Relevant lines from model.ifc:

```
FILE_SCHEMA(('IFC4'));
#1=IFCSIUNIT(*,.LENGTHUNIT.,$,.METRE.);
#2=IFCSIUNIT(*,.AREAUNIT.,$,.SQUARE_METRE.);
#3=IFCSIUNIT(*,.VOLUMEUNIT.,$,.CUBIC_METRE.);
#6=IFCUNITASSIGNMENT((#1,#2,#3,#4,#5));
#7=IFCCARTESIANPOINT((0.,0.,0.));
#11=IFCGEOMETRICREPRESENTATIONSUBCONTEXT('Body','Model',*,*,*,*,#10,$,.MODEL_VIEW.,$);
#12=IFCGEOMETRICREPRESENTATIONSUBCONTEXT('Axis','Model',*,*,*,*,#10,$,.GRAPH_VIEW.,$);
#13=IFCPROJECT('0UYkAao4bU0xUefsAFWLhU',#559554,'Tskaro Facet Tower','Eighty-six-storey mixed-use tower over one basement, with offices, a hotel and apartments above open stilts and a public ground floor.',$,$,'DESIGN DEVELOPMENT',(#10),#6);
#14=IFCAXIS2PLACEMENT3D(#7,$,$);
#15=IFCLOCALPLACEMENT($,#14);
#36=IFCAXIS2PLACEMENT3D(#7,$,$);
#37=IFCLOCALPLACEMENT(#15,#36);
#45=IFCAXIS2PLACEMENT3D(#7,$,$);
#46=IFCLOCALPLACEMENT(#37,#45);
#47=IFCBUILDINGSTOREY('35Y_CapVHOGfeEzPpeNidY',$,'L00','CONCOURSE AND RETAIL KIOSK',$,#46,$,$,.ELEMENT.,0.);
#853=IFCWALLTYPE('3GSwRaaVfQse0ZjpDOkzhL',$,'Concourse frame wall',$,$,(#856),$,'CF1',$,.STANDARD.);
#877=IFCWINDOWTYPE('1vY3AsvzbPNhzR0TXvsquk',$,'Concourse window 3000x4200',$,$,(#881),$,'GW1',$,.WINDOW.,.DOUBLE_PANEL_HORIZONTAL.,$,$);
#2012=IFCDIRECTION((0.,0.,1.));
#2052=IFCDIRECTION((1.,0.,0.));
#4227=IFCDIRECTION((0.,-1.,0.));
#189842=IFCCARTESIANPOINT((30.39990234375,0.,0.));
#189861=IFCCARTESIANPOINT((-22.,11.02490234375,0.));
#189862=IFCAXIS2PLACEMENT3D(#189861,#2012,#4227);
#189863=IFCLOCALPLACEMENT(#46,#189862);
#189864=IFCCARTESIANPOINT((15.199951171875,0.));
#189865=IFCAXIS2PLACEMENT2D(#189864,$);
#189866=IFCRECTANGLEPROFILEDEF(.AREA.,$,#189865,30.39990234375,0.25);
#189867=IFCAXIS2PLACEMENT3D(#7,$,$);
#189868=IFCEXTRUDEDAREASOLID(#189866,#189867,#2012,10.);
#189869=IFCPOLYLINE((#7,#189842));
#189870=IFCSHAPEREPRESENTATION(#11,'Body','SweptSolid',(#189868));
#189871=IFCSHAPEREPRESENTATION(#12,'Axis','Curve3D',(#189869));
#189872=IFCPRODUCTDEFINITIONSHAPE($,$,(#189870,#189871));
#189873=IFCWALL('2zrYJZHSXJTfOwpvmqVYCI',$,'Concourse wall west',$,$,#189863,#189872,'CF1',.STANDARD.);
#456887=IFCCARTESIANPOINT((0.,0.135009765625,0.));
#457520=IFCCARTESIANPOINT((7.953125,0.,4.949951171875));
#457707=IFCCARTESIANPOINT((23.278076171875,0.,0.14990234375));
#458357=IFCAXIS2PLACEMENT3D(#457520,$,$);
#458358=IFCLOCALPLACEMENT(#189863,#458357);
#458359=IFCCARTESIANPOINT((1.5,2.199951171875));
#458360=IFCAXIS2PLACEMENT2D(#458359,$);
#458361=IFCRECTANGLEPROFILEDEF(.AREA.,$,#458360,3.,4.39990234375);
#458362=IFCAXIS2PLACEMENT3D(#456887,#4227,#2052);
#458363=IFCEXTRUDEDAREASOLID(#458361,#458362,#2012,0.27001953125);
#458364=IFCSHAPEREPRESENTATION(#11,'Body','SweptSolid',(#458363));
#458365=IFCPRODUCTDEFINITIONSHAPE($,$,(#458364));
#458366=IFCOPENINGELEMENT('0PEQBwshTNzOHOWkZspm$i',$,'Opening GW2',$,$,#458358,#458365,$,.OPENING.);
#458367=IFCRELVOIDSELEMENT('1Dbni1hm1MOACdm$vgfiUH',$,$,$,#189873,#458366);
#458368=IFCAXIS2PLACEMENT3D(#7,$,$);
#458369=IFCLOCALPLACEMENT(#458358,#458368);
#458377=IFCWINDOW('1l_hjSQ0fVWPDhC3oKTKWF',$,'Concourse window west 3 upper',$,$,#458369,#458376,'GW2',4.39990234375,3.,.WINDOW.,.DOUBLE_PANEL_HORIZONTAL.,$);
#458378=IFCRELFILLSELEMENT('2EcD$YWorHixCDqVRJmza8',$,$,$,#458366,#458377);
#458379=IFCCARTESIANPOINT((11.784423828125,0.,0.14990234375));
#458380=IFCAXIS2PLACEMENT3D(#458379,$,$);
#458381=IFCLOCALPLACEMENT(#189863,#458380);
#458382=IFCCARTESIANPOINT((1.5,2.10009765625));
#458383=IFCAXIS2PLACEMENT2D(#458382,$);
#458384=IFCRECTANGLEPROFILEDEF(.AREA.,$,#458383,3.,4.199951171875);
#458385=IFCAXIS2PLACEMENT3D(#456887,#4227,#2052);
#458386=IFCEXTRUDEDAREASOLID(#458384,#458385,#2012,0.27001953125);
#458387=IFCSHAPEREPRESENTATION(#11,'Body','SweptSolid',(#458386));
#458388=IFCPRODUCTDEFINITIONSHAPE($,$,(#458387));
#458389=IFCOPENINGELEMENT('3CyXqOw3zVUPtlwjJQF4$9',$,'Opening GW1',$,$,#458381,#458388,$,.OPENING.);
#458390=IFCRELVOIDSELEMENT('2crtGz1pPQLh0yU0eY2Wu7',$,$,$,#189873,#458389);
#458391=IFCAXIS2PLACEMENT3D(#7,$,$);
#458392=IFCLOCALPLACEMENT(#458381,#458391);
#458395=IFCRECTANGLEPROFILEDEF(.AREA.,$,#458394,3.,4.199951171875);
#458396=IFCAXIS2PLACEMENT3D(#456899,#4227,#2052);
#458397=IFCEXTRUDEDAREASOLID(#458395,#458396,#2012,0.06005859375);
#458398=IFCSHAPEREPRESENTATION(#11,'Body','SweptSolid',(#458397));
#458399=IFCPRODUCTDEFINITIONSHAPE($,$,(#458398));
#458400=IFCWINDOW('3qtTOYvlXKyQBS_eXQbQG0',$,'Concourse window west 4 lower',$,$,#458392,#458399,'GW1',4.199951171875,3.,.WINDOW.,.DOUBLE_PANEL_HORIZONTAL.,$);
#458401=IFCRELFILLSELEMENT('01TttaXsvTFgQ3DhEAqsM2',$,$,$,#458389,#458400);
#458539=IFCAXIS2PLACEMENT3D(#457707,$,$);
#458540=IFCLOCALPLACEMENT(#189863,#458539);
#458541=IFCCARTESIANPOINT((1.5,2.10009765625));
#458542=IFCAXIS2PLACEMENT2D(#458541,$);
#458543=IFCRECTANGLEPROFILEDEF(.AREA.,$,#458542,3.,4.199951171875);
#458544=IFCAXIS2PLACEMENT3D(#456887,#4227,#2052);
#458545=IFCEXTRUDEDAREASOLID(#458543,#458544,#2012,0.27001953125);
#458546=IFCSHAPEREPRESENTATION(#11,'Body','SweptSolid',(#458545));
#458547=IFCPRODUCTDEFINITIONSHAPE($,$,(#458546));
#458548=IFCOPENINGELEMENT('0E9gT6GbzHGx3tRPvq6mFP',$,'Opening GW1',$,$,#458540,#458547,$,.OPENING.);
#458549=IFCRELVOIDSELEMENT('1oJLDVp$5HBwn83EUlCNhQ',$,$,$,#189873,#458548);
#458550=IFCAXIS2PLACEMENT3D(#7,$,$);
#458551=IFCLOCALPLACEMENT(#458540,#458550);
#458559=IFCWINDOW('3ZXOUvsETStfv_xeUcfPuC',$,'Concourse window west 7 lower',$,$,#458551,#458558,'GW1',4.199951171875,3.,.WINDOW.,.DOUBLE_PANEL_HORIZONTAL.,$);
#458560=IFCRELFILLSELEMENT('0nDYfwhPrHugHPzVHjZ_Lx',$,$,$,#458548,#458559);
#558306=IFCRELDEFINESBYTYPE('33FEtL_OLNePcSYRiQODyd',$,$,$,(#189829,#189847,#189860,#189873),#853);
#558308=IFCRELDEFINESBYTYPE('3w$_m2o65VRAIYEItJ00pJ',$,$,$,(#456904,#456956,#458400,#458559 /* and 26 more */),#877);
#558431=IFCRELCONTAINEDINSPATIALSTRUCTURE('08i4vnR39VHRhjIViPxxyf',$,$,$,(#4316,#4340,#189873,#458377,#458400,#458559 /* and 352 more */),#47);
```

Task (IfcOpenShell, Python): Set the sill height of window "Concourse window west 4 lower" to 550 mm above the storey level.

```python
import numpy as np
import ifcopenshell
import ifcopenshell.api.geometry
import ifcopenshell.geom
import ifcopenshell.util.element
import ifcopenshell.util.placement
import ifcopenshell.util.shape
import ifcopenshell.util.unit

model = ifcopenshell.open("model.ifc")
unit_scale = ifcopenshell.util.unit.calculate_unit_scale(model)

window = model.by_guid("3qtTOYvlXKyQBS_eXQbQG0")
opening = window.FillsVoids[0].RelatingOpeningElement
storey = ifcopenshell.util.element.get_container(window, ifc_class="IfcBuildingStorey")
level = ifcopenshell.util.placement.get_local_placement(storey.ObjectPlacement)[2, 3]

# The opening's origin need not be at the sill, so measure its lowest point.
shape = ifcopenshell.geom.create_shape(ifcopenshell.geom.settings(), opening)
bottom = ifcopenshell.util.shape.get_shape_bottom_elevation(shape, shape.geometry) / unit_scale
dz = level + 0.55 / unit_scale - bottom

shift = np.array([0.0, 0.0, dz])
# The window is placed relative to its opening, so it follows when the opening moves.
matrix = ifcopenshell.util.placement.get_local_placement(opening.ObjectPlacement)
matrix[:3, 3] += shift
ifcopenshell.api.geometry.edit_object_placement(
    model, product=opening, matrix=matrix, is_si=False, should_transform_children=True
)

print(f"moved by {dz * unit_scale:+.3f} m")

model.write("model-out.ifc")
```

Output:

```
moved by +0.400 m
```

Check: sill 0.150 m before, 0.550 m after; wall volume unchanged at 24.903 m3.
